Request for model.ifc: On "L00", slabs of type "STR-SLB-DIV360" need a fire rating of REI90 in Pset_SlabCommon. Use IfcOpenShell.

First a look at what the model holds.

```python
import ifcopenshell
import ifcopenshell.util.element

model = ifcopenshell.open("model.ifc")
print(model.schema)
storey = next(s for s in model.by_type("IfcBuildingStorey") if s.Name == "L00")
slabs = [e for e in ifcopenshell.util.element.get_decomposition(storey) if e.is_a("IfcSlab")]
seen = {}
for e in slabs:
    element_type = ifcopenshell.util.element.get_type(e)
    key = (element_type.Name if element_type != e and element_type else None, ifcopenshell.util.element.get_pset(e, "Pset_SlabCommon", "FireRating"))
    seen[key] = seen.get(key, 0) + 1
for (name, value), count in sorted(seen.items(), key=str):
    print(count, "x", name, "|", value)
```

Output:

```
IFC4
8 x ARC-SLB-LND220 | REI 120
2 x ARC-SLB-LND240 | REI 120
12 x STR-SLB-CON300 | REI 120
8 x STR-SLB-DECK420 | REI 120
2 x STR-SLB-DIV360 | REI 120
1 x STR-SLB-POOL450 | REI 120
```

```python
import ifcopenshell
import ifcopenshell.api.pset
import ifcopenshell.util.element

model = ifcopenshell.open("model.ifc")

storey = next(s for s in model.by_type("IfcBuildingStorey") if s.Name == "L00")
slabs = [e for e in ifcopenshell.util.element.get_decomposition(storey) if e.is_a("IfcSlab")]

count = 0
for e in slabs:
    element_type = ifcopenshell.util.element.get_type(e)
    if element_type in (None, e) or element_type.Name != "STR-SLB-DIV360":
        continue
    # add_pset returns the element's existing set when there is one.
    pset = ifcopenshell.api.pset.add_pset(model, product=e, name="Pset_SlabCommon")
    ifcopenshell.api.pset.edit_pset(model, pset=pset, properties={"FireRating": "REI90"})
    count += 1

print(count, "slabs updated")

model.write("model_updated.ifc")
```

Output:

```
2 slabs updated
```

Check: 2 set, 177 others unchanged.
